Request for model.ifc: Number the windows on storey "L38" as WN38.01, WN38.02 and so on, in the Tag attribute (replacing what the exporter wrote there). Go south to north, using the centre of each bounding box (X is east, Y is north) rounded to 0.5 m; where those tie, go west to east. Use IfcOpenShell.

First a look at what the model holds.

```python
import ifcopenshell
import ifcopenshell.util.element
import ifcopenshell.util.placement

model = ifcopenshell.open("model.ifc")
print(model.schema)
storey = next(s for s in model.by_type("IfcBuildingStorey") if s.Name == "L38")
windows = [e for e in ifcopenshell.util.element.get_decomposition(storey) if e.is_a("IfcWindow")]
for e in sorted(windows, key=lambda e: e.id()):
    origin = ifcopenshell.util.placement.get_local_placement(e.ObjectPlacement)[:3, 3]
    print(e.id(), e.Tag, e.Name, origin.round(2) + 0.0, sep=" | ")
```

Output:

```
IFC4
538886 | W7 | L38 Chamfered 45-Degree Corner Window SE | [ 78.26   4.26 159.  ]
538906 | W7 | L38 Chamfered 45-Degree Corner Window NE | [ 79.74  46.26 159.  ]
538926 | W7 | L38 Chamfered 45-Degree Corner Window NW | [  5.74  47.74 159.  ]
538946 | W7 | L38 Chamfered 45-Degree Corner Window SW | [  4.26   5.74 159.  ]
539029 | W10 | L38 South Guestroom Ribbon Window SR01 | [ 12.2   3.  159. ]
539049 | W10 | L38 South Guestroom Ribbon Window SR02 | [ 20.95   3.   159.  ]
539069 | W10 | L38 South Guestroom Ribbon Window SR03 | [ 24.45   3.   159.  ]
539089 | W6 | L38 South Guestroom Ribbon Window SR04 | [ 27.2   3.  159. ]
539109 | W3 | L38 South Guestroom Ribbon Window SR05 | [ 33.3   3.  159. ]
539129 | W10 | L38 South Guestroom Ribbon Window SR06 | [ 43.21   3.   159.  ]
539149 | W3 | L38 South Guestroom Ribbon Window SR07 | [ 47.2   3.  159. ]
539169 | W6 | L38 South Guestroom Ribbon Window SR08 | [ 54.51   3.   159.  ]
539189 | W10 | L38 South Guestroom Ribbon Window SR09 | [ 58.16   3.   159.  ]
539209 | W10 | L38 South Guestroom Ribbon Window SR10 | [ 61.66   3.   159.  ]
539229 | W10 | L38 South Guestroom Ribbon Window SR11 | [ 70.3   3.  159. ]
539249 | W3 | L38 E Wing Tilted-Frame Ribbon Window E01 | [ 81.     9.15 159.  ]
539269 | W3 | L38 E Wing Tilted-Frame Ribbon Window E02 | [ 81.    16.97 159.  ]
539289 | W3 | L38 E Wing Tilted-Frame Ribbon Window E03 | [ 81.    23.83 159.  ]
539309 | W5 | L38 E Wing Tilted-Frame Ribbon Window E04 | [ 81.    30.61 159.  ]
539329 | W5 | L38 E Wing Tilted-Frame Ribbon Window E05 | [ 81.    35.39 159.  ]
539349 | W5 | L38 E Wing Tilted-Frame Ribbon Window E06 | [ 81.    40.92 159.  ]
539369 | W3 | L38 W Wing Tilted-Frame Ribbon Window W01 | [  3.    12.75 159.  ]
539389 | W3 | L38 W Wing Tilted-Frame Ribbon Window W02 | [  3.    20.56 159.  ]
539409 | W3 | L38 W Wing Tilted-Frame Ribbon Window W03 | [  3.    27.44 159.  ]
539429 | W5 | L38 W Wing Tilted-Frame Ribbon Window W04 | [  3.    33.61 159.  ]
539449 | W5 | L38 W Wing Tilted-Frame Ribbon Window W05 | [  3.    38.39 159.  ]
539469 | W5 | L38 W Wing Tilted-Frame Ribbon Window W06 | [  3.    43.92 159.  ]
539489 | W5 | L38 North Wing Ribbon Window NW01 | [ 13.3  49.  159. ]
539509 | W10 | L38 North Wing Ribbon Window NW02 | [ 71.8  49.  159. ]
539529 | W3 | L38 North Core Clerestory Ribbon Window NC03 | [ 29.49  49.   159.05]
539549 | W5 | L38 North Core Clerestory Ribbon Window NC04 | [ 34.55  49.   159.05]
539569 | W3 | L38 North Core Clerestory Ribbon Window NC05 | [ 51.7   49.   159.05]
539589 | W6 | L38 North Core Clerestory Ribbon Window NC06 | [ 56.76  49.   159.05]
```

```python
import ifcopenshell
import ifcopenshell.geom
import ifcopenshell.util.element
import ifcopenshell.util.shape

model = ifcopenshell.open("model.ifc")
settings = ifcopenshell.geom.settings()
settings.set("use-world-coords", True)


def centre(element):
    shape = ifcopenshell.geom.create_shape(settings, element)
    return ifcopenshell.util.shape.get_bbox_centroid(shape.geometry)


storey = next(s for s in model.by_type("IfcBuildingStorey") if s.Name == "L38")
windows = [e for e in ifcopenshell.util.element.get_decomposition(storey) if e.is_a("IfcWindow")]

# Insertion points can sit at a corner or the storey origin, so sort by the geometry (in metres).
centres = {e: centre(e) for e in windows}
windows.sort(key=lambda e: (round(centres[e][1] / 0.5), centres[e][0]))

for i, e in enumerate(windows, start=1):
    number = f"WN38.{i:02d}"
    e.Tag = number
    print(e.id(), number)

model.write("model_rev.ifc")
```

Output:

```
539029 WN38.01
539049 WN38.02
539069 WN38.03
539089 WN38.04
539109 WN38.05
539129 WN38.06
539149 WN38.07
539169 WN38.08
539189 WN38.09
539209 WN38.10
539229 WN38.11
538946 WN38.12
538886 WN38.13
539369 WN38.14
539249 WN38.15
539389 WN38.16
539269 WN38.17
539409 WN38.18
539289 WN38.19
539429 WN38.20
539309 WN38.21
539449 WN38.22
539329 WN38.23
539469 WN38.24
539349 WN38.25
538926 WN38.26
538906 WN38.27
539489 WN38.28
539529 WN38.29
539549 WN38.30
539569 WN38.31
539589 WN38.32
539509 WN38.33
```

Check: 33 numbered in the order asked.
